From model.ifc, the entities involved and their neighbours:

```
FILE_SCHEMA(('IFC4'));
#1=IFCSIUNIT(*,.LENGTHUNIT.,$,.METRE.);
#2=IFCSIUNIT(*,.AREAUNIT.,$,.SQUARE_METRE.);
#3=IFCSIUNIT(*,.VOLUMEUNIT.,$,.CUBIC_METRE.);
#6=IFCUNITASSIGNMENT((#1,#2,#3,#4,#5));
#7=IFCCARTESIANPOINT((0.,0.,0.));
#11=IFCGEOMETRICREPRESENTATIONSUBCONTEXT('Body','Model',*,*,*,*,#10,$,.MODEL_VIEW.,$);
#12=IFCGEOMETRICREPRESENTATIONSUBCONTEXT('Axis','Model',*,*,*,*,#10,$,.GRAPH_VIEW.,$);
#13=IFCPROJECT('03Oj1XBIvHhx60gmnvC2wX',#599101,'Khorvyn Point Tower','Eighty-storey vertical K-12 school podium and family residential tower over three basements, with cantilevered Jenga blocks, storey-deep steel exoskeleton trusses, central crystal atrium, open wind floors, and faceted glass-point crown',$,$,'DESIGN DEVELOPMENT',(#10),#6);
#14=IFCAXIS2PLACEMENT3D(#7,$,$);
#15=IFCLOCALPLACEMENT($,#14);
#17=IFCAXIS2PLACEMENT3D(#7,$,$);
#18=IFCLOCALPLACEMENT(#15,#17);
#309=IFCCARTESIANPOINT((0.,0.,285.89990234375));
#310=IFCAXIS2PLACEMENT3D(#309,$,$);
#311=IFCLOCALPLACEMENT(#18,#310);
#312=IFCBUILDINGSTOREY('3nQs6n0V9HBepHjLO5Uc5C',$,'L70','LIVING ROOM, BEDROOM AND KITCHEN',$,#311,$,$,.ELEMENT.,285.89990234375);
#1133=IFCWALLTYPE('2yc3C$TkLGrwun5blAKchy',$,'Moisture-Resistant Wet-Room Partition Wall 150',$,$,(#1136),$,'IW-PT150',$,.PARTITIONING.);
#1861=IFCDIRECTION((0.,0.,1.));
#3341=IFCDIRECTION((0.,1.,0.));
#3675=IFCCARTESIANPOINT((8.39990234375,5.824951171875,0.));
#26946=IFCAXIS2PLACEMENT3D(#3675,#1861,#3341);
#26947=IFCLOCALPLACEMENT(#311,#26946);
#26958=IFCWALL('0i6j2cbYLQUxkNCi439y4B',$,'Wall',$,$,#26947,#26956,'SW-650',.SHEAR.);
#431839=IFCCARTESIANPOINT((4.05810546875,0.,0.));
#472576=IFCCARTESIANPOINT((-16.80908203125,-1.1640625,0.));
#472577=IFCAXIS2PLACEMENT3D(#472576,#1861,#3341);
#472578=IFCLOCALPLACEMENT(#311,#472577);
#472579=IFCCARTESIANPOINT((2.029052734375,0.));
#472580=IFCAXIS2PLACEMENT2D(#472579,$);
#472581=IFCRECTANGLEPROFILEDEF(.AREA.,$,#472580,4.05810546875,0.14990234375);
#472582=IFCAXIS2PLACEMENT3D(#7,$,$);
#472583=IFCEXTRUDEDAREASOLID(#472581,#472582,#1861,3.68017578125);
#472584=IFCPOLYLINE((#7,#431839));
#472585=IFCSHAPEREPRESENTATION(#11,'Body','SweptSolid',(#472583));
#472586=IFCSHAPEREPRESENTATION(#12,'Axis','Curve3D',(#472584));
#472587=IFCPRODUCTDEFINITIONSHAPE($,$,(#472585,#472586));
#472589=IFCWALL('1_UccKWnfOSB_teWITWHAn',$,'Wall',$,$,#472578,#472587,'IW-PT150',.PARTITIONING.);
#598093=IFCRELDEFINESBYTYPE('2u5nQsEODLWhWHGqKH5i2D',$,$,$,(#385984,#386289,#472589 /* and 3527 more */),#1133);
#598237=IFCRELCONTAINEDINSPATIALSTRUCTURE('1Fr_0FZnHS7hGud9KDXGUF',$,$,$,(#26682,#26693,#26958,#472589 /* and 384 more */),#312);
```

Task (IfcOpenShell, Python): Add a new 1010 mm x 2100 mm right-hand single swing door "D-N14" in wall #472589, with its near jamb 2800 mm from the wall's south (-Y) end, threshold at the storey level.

```python
import numpy as np
import ifcopenshell
import ifcopenshell.api.feature
import ifcopenshell.api.geometry
import ifcopenshell.api.root
import ifcopenshell.api.spatial
import ifcopenshell.geom
import ifcopenshell.util.element
import ifcopenshell.util.placement
import ifcopenshell.util.representation
import ifcopenshell.util.shape
import ifcopenshell.util.unit

model = ifcopenshell.open("model.ifc")
unit_scale = ifcopenshell.util.unit.calculate_unit_scale(model)
settings = ifcopenshell.geom.settings()


def volume(element):
    """Net volume in cubic metres, openings subtracted."""
    shape = ifcopenshell.geom.create_shape(settings, element)
    return ifcopenshell.util.shape.get_volume(shape.geometry)


wall = model.by_id(472589)
storey = ifcopenshell.util.element.get_container(wall, ifc_class="IfcBuildingStorey")
context = ifcopenshell.util.representation.get_context(model, "Model", "Body", "MODEL_VIEW")
before = volume(wall)

width, height, from_end, sill = 1.01, 2.1, 2.8, 0.0  # metres

# The wall runs along its own X axis, and the end named is its -X end.
wall_shape = ifcopenshell.geom.create_shape(settings, wall)
x, y, z = ifcopenshell.util.shape.get_vertices(wall_shape.geometry).T
start = x.min() + from_end
face, thickness = float(y.min()), float(y.max() - y.min())
wall_matrix = ifcopenshell.util.placement.get_local_placement(wall.ObjectPlacement)
level = ifcopenshell.util.placement.get_local_placement(storey.ObjectPlacement)[2, 3]


def in_wall(x, y):
    """Placement at x, y metres in the wall's axes, at sill height."""
    matrix = wall_matrix.copy()
    matrix[:, 3] = wall_matrix @ np.array([x / unit_scale, y / unit_scale, 0.0, 1.0])
    matrix[2, 3] = level + sill / unit_scale
    return matrix


# Opening: a box that overshoots both wall faces by 50 mm.
opening = ifcopenshell.api.root.create_entity(model, ifc_class="IfcOpeningElement", predefined_type="OPENING")
box = ifcopenshell.api.geometry.add_wall_representation(
    model, context=context, length=width, height=height, thickness=thickness + 0.1
)
ifcopenshell.api.geometry.assign_representation(model, product=opening, representation=box)
ifcopenshell.api.geometry.edit_object_placement(model, product=opening, matrix=in_wall(start, face - 0.05), is_si=False)
ifcopenshell.api.feature.add_feature(model, feature=opening, element=wall)

door = ifcopenshell.api.root.create_entity(model, ifc_class="IfcDoor", name="D-N14", predefined_type="DOOR")
door.OverallWidth, door.OverallHeight = width / unit_scale, height / unit_scale
door.OperationType = "SINGLE_SWING_RIGHT"
body = ifcopenshell.api.geometry.add_door_representation(
    model,
    context=context,
    overall_width=door.OverallWidth,
    overall_height=door.OverallHeight,
    operation_type="SINGLE_SWING_RIGHT",
    lining_properties={"LiningDepth": thickness / unit_scale, "ThresholdDepth": thickness / unit_scale},
)
ifcopenshell.api.geometry.assign_representation(model, product=door, representation=body)
ifcopenshell.api.spatial.assign_container(model, products=[door], relating_structure=storey)
ifcopenshell.api.feature.add_filling(model, opening=opening, element=door)

# The lining spans the wall, so the door starts at the wall face.
ifcopenshell.api.geometry.edit_object_placement(model, product=door, matrix=in_wall(start, face), is_si=False)

after = volume(wall)

print(f"wall volume {before:.3f} -> {after:.3f} m3")

model.write("model-out.ifc")
```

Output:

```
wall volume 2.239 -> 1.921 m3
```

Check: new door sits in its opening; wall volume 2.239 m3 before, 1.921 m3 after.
